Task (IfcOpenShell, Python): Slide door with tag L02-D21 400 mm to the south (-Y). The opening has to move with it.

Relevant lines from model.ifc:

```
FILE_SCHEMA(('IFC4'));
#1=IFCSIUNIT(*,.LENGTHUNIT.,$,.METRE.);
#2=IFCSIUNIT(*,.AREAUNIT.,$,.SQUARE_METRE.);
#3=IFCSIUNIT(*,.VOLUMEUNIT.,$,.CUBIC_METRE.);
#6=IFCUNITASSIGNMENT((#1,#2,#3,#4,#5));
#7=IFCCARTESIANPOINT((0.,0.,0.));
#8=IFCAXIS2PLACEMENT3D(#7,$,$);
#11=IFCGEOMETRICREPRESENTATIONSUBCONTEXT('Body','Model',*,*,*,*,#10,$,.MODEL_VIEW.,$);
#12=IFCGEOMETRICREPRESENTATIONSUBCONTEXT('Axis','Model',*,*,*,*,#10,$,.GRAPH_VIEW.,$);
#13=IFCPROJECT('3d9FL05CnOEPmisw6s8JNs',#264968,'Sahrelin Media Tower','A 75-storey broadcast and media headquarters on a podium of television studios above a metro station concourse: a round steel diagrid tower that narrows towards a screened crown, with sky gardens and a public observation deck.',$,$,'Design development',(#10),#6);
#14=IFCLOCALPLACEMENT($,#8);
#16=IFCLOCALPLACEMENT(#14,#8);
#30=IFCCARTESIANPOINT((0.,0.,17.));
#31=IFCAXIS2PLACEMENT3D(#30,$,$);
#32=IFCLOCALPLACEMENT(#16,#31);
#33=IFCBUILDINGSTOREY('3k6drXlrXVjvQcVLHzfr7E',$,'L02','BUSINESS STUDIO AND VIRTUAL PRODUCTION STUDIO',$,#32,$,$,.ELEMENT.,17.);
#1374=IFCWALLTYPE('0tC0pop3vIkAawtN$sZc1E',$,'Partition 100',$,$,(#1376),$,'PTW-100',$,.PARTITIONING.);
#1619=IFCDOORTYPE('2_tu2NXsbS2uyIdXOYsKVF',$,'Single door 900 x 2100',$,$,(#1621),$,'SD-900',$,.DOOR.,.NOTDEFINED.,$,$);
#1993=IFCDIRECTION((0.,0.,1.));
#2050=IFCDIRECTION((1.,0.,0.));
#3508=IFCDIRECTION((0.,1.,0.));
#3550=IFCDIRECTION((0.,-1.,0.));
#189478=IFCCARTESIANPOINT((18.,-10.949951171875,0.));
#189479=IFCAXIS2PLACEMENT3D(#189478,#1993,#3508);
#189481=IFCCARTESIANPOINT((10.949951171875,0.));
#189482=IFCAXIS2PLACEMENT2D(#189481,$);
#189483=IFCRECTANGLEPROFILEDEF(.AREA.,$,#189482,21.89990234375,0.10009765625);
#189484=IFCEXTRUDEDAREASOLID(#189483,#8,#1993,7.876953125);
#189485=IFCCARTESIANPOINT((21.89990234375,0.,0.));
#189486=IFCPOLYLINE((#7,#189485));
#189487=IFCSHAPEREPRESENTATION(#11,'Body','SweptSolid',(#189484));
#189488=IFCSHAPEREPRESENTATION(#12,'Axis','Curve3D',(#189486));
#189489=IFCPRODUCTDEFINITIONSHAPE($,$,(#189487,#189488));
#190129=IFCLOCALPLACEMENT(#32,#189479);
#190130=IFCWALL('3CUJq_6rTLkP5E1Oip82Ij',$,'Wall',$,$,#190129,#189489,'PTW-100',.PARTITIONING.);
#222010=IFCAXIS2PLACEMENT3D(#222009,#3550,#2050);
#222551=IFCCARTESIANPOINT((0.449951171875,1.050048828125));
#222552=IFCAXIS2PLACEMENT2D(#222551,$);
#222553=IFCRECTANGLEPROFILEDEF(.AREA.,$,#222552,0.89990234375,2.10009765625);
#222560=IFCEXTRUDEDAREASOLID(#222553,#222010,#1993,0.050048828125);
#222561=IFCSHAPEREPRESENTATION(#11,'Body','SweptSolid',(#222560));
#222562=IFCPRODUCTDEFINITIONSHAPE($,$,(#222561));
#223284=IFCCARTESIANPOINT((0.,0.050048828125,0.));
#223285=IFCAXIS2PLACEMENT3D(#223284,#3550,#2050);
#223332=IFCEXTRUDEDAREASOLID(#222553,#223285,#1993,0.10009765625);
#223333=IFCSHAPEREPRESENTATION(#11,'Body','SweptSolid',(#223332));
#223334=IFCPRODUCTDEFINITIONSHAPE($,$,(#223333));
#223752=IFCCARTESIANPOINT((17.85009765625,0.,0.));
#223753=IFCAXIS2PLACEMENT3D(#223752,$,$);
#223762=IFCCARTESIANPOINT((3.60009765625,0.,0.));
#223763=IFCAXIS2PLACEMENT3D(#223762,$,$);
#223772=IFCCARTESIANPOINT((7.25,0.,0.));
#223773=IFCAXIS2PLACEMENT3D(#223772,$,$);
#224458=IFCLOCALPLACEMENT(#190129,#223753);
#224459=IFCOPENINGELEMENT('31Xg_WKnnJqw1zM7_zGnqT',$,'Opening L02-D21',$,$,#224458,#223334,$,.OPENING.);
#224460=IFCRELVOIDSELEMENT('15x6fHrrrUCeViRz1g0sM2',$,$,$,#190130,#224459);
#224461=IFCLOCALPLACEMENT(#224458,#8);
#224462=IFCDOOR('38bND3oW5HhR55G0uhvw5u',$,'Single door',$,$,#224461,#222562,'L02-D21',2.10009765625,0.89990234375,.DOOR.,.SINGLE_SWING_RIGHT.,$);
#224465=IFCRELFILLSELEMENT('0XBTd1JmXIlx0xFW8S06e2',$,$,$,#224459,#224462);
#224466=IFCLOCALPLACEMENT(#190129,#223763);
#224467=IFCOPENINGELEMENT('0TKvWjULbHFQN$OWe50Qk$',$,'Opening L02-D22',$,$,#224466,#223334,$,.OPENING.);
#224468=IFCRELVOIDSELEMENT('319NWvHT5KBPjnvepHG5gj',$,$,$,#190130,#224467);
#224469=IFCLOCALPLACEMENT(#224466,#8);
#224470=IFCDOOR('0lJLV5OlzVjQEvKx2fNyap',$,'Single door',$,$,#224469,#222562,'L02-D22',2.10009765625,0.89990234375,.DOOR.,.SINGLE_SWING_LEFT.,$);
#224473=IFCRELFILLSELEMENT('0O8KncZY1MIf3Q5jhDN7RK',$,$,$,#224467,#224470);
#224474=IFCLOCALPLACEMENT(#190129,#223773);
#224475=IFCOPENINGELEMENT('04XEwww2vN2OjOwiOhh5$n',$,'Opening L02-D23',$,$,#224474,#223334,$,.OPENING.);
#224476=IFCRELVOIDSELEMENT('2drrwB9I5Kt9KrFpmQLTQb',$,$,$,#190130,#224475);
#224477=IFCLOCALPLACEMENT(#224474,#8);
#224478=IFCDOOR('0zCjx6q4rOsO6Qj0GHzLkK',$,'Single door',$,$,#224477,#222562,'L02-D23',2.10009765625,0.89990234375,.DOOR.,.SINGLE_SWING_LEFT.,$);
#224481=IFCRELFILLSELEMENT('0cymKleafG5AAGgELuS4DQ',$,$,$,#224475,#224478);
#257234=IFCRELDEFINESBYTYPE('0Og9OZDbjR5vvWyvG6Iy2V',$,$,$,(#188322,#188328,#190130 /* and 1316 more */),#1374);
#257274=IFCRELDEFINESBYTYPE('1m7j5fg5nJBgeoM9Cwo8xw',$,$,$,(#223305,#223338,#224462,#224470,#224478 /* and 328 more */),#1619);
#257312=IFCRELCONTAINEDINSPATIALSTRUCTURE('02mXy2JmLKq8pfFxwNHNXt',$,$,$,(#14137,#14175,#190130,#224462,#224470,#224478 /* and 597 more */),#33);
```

```python
import ifcopenshell
import ifcopenshell.api.geometry
import ifcopenshell.util.placement
import ifcopenshell.util.unit

model = ifcopenshell.open("model.ifc")
unit_scale = ifcopenshell.util.unit.calculate_unit_scale(model)

door = model.by_guid("38bND3oW5HhR55G0uhvw5u")
opening = door.FillsVoids[0].RelatingOpeningElement
wall = opening.VoidsElements[0].RelatingBuildingElement

wall_matrix = ifcopenshell.util.placement.get_local_placement(wall.ObjectPlacement)
shift = wall_matrix[:3, 0] * -0.4 / unit_scale
before = ifcopenshell.util.placement.get_local_placement(door.ObjectPlacement)[:3, 3].copy()

# The door is placed relative to its opening, so it follows when the opening moves.
matrix = ifcopenshell.util.placement.get_local_placement(opening.ObjectPlacement)
matrix[:3, 3] += shift
ifcopenshell.api.geometry.edit_object_placement(
    model, product=opening, matrix=matrix, is_si=False, should_transform_children=True
)

after = ifcopenshell.util.placement.get_local_placement(door.ObjectPlacement)[:3, 3]
print("door moved by", (after - before).round(3) + 0.0)

model.write("model_updated.ifc")
```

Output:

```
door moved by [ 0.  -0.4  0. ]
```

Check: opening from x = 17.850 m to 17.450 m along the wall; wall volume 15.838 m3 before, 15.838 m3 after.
